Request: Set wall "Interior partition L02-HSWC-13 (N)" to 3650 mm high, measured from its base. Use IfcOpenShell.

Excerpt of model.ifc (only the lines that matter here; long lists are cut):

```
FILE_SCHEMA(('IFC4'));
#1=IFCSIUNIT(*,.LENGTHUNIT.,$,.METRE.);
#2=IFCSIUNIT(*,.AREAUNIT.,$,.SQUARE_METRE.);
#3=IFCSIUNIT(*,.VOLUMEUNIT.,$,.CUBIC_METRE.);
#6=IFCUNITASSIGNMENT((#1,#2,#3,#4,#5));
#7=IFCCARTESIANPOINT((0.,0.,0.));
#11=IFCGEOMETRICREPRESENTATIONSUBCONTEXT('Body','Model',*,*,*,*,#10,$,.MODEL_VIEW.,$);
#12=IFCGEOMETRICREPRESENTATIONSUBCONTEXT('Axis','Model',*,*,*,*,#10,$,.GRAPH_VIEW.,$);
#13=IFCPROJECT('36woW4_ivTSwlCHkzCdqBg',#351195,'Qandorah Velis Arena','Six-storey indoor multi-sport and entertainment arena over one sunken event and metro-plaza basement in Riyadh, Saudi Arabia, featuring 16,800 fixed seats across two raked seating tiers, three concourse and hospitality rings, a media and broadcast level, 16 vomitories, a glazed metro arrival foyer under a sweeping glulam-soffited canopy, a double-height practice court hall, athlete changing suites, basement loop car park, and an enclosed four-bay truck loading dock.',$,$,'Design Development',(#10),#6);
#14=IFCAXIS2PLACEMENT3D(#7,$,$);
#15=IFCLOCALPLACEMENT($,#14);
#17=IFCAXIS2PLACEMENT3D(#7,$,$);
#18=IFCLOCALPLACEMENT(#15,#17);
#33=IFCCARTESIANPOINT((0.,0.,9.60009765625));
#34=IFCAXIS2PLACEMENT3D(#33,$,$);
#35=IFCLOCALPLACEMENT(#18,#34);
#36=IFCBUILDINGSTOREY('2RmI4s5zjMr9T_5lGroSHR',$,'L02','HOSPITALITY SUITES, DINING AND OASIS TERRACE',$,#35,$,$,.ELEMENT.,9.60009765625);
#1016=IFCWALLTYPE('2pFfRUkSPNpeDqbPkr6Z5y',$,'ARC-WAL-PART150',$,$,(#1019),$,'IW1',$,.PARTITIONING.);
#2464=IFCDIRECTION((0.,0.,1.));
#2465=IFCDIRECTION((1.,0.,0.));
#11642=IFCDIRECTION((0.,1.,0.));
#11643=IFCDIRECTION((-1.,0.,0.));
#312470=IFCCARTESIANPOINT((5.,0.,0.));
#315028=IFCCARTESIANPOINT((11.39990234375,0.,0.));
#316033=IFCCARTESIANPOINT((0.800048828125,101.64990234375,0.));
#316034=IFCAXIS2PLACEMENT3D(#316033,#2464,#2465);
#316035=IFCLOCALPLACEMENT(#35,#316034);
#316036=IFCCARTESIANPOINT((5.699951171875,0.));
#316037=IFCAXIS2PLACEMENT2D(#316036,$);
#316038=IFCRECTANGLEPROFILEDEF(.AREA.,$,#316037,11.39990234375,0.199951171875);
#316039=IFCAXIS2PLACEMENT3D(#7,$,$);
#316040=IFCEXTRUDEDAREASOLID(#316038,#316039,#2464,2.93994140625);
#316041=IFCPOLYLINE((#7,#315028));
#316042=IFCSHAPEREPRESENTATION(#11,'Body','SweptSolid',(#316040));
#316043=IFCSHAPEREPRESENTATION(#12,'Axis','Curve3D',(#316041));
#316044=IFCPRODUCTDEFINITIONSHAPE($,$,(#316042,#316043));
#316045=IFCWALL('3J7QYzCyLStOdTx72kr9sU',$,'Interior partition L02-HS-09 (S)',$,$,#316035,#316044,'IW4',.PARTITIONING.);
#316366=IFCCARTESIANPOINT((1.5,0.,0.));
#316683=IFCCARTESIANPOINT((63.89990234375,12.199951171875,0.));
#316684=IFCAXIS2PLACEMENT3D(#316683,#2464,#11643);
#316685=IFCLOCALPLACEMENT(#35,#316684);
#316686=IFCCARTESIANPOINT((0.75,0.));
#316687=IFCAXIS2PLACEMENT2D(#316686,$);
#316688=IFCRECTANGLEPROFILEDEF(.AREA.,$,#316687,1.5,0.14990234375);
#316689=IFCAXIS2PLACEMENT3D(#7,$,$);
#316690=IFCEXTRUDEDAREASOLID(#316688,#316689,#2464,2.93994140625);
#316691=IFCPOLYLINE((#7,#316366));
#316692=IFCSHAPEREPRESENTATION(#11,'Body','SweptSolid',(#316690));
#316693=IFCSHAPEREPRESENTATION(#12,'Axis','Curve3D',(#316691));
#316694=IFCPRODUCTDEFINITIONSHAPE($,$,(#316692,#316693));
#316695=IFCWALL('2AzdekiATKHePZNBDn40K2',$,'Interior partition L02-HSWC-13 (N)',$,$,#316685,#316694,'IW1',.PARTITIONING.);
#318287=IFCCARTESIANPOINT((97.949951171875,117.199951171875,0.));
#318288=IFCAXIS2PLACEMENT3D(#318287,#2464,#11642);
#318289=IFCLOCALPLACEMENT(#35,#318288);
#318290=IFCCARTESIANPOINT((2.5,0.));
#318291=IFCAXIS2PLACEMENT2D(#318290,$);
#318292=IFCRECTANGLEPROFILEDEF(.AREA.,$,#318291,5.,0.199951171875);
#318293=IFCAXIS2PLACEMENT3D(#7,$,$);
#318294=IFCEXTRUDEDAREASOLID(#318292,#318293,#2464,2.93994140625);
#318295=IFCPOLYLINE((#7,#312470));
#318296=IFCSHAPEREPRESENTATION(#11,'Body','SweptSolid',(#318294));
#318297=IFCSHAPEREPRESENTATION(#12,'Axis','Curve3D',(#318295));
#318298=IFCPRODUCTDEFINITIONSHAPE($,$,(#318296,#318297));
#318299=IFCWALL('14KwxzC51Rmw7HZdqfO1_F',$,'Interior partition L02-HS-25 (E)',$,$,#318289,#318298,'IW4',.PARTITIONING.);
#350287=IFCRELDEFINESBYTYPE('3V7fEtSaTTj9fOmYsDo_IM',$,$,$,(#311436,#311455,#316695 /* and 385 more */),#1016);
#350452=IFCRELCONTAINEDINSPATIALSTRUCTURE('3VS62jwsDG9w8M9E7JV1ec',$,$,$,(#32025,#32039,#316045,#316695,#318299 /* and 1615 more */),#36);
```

```python
import ifcopenshell
import ifcopenshell.geom
import ifcopenshell.util.representation
import ifcopenshell.util.shape
import ifcopenshell.util.unit

model = ifcopenshell.open("model.ifc")
unit_scale = ifcopenshell.util.unit.calculate_unit_scale(model)
settings = ifcopenshell.geom.settings()


def volume(element):
    """Net volume in cubic metres, openings subtracted."""
    shape = ifcopenshell.geom.create_shape(settings, element)
    return ifcopenshell.util.shape.get_volume(shape.geometry)


wall = model.by_guid("2AzdekiATKHePZNBDn40K2")
before = volume(wall)

body = ifcopenshell.util.representation.get_representation(wall, "Model", "Body")
solid = body.Items[0]
old_height = solid.Depth
solid.Depth = 3.65 / unit_scale
after = volume(wall)

print(f"height {old_height:g} -> {solid.Depth:g}, volume {before:.3f} -> {after:.3f} m3")

model.write("model_updated.ifc")
```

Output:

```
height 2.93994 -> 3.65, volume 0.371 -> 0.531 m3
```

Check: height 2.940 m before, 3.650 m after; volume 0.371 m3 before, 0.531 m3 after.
